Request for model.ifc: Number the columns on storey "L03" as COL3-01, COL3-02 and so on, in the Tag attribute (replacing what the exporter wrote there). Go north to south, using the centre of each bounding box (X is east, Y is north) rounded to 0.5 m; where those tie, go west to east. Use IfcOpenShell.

First a look at what the model holds.

```python
import ifcopenshell
import ifcopenshell.util.element
import ifcopenshell.util.placement

model = ifcopenshell.open("model.ifc")
print(model.schema)
storey = next(s for s in model.by_type("IfcBuildingStorey") if s.Name == "L03")
columns = [e for e in ifcopenshell.util.element.get_decomposition(storey) if e.is_a("IfcColumn")]
for e in sorted(columns, key=lambda e: e.id()):
    origin = ifcopenshell.util.placement.get_local_placement(e.ObjectPlacement)[:3, 3]
    print(e.id(), e.Tag, e.Name, origin.round(2) + 0.0, sep=" | ")
```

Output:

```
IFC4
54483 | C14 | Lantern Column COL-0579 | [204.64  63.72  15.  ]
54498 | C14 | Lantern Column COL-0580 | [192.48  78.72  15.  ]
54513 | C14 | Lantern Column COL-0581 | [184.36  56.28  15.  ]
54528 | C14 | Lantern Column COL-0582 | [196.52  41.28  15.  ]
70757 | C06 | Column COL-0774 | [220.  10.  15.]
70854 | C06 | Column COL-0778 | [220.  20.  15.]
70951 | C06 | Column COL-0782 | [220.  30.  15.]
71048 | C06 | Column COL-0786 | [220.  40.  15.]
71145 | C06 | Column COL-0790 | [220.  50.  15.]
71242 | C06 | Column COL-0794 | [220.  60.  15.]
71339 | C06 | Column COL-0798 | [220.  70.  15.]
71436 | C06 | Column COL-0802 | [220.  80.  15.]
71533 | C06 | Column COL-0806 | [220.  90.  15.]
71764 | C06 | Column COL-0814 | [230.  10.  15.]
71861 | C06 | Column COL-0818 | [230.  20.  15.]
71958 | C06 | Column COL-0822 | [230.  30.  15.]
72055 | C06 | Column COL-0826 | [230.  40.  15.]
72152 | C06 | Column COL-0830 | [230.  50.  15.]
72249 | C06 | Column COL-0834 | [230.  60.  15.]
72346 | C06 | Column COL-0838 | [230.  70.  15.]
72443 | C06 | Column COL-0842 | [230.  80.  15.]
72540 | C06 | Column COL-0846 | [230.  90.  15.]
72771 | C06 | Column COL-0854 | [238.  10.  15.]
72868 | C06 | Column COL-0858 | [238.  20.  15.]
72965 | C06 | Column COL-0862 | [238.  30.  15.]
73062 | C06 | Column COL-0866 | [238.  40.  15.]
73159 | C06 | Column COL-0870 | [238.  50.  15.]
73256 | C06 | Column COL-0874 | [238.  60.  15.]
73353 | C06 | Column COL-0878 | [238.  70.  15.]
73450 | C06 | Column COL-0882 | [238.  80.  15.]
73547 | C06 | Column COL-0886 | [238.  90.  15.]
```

```python
import ifcopenshell
import ifcopenshell.geom
import ifcopenshell.util.element
import ifcopenshell.util.shape

model = ifcopenshell.open("model.ifc")
settings = ifcopenshell.geom.settings()
settings.set("use-world-coords", True)


def centre(element):
    shape = ifcopenshell.geom.create_shape(settings, element)
    return ifcopenshell.util.shape.get_bbox_centroid(shape.geometry)


storey = next(s for s in model.by_type("IfcBuildingStorey") if s.Name == "L03")
columns = [e for e in ifcopenshell.util.element.get_decomposition(storey) if e.is_a("IfcColumn")]

# Insertion points can sit at a corner or the storey origin, so sort by the geometry (in metres).
centres = {e: centre(e) for e in columns}
columns.sort(key=lambda e: (-round(centres[e][1] / 0.5), centres[e][0]))

for i, e in enumerate(columns, start=1):
    number = f"COL3-{i:02d}"
    e.Tag = number
    print(e.id(), number)

model.write("model_edited.ifc")
```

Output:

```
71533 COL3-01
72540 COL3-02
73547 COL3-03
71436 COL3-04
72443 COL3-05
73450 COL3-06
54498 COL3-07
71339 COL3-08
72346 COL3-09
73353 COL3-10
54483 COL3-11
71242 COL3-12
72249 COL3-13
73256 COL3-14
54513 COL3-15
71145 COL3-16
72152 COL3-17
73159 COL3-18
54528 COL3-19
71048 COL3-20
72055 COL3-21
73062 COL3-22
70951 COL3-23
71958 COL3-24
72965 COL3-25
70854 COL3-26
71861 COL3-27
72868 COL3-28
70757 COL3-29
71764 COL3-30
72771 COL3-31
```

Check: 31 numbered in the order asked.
